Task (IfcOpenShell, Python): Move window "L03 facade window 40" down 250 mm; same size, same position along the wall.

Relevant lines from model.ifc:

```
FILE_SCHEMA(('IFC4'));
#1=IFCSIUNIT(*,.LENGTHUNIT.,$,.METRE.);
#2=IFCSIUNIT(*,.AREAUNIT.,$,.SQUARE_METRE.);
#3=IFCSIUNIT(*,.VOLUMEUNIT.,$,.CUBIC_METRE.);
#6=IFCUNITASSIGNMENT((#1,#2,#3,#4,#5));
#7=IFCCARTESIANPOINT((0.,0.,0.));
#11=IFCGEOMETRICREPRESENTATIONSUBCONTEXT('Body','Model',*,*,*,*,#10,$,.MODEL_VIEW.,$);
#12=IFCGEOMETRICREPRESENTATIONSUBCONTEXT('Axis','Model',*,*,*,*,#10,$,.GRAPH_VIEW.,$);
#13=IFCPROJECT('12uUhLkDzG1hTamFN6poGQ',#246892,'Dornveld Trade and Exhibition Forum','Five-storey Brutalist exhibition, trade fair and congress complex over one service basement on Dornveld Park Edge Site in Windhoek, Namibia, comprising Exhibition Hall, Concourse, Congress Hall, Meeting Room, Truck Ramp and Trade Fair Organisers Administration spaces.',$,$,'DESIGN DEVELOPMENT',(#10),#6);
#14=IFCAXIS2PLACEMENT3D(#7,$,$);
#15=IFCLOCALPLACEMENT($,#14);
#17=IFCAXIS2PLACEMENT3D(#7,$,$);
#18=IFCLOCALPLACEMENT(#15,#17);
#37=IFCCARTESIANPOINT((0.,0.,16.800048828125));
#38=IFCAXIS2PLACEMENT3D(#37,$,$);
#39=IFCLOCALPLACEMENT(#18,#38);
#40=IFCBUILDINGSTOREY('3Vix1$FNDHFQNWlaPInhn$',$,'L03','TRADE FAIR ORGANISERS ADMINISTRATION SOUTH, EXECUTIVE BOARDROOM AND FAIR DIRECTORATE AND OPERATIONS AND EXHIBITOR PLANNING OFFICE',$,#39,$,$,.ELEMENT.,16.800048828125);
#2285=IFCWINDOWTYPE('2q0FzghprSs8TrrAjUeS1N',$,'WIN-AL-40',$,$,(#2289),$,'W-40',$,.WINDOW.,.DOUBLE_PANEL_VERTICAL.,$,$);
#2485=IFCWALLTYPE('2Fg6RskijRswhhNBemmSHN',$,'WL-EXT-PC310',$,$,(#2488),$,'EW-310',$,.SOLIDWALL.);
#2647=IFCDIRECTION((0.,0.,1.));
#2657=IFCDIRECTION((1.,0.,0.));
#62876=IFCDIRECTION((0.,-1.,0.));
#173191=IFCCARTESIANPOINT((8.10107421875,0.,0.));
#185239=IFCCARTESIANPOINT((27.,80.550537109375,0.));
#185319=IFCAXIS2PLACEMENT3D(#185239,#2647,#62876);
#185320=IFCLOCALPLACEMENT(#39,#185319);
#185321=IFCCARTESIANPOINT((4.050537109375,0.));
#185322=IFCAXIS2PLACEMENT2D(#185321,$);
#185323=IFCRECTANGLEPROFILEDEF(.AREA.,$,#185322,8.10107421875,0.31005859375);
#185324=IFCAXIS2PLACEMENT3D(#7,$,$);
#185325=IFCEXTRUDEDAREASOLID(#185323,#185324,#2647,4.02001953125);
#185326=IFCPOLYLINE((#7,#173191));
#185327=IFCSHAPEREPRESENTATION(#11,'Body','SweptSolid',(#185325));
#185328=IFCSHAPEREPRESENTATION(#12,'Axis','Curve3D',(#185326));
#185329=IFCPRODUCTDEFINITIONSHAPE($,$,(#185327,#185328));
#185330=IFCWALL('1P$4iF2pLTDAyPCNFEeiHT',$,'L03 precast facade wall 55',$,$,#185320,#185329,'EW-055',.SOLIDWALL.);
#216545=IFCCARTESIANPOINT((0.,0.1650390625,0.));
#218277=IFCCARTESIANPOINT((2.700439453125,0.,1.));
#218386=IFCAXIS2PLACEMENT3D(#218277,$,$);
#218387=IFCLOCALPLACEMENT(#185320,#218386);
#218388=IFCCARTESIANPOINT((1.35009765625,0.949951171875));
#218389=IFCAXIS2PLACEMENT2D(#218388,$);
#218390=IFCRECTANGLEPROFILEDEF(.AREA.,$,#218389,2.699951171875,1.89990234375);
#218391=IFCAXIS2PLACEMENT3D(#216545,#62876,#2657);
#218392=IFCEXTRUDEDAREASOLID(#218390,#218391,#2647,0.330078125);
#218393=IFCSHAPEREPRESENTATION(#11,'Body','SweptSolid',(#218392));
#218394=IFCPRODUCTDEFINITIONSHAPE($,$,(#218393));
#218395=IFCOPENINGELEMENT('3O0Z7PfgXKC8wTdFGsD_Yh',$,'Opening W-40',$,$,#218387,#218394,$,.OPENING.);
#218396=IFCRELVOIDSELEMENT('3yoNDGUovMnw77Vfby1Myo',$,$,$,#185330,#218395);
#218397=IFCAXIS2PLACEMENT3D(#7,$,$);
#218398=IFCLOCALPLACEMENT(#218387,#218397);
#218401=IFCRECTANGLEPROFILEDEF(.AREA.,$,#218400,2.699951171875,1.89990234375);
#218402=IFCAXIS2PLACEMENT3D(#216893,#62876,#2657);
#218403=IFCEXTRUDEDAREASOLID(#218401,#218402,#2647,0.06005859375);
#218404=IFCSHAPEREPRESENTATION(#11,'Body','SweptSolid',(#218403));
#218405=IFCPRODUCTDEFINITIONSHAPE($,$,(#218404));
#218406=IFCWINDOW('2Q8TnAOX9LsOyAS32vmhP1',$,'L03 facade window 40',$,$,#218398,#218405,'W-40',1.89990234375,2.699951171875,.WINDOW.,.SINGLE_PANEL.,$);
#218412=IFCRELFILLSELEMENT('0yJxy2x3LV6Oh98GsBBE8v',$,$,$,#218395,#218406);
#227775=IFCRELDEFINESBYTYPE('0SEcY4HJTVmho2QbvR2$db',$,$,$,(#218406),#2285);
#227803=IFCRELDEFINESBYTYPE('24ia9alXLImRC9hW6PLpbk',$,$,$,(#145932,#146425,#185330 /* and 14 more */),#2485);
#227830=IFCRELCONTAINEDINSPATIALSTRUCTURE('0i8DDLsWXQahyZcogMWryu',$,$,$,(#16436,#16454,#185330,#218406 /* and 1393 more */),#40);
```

```python
import numpy as np
import ifcopenshell
import ifcopenshell.api.geometry
import ifcopenshell.util.placement
import ifcopenshell.util.unit

model = ifcopenshell.open("model.ifc")
unit_scale = ifcopenshell.util.unit.calculate_unit_scale(model)

window = model.by_guid("2Q8TnAOX9LsOyAS32vmhP1")
opening = window.FillsVoids[0].RelatingOpeningElement
dz = -0.25 / unit_scale

shift = np.array([0.0, 0.0, dz])
# The window is placed relative to its opening, so it follows when the opening moves.
matrix = ifcopenshell.util.placement.get_local_placement(opening.ObjectPlacement)
matrix[:3, 3] += shift
ifcopenshell.api.geometry.edit_object_placement(
    model, product=opening, matrix=matrix, is_si=False, should_transform_children=True
)

print(f"moved by {dz * unit_scale:+.3f} m")

model.write("model_rev.ifc")
```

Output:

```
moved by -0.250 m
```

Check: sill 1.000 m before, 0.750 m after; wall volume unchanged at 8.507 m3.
